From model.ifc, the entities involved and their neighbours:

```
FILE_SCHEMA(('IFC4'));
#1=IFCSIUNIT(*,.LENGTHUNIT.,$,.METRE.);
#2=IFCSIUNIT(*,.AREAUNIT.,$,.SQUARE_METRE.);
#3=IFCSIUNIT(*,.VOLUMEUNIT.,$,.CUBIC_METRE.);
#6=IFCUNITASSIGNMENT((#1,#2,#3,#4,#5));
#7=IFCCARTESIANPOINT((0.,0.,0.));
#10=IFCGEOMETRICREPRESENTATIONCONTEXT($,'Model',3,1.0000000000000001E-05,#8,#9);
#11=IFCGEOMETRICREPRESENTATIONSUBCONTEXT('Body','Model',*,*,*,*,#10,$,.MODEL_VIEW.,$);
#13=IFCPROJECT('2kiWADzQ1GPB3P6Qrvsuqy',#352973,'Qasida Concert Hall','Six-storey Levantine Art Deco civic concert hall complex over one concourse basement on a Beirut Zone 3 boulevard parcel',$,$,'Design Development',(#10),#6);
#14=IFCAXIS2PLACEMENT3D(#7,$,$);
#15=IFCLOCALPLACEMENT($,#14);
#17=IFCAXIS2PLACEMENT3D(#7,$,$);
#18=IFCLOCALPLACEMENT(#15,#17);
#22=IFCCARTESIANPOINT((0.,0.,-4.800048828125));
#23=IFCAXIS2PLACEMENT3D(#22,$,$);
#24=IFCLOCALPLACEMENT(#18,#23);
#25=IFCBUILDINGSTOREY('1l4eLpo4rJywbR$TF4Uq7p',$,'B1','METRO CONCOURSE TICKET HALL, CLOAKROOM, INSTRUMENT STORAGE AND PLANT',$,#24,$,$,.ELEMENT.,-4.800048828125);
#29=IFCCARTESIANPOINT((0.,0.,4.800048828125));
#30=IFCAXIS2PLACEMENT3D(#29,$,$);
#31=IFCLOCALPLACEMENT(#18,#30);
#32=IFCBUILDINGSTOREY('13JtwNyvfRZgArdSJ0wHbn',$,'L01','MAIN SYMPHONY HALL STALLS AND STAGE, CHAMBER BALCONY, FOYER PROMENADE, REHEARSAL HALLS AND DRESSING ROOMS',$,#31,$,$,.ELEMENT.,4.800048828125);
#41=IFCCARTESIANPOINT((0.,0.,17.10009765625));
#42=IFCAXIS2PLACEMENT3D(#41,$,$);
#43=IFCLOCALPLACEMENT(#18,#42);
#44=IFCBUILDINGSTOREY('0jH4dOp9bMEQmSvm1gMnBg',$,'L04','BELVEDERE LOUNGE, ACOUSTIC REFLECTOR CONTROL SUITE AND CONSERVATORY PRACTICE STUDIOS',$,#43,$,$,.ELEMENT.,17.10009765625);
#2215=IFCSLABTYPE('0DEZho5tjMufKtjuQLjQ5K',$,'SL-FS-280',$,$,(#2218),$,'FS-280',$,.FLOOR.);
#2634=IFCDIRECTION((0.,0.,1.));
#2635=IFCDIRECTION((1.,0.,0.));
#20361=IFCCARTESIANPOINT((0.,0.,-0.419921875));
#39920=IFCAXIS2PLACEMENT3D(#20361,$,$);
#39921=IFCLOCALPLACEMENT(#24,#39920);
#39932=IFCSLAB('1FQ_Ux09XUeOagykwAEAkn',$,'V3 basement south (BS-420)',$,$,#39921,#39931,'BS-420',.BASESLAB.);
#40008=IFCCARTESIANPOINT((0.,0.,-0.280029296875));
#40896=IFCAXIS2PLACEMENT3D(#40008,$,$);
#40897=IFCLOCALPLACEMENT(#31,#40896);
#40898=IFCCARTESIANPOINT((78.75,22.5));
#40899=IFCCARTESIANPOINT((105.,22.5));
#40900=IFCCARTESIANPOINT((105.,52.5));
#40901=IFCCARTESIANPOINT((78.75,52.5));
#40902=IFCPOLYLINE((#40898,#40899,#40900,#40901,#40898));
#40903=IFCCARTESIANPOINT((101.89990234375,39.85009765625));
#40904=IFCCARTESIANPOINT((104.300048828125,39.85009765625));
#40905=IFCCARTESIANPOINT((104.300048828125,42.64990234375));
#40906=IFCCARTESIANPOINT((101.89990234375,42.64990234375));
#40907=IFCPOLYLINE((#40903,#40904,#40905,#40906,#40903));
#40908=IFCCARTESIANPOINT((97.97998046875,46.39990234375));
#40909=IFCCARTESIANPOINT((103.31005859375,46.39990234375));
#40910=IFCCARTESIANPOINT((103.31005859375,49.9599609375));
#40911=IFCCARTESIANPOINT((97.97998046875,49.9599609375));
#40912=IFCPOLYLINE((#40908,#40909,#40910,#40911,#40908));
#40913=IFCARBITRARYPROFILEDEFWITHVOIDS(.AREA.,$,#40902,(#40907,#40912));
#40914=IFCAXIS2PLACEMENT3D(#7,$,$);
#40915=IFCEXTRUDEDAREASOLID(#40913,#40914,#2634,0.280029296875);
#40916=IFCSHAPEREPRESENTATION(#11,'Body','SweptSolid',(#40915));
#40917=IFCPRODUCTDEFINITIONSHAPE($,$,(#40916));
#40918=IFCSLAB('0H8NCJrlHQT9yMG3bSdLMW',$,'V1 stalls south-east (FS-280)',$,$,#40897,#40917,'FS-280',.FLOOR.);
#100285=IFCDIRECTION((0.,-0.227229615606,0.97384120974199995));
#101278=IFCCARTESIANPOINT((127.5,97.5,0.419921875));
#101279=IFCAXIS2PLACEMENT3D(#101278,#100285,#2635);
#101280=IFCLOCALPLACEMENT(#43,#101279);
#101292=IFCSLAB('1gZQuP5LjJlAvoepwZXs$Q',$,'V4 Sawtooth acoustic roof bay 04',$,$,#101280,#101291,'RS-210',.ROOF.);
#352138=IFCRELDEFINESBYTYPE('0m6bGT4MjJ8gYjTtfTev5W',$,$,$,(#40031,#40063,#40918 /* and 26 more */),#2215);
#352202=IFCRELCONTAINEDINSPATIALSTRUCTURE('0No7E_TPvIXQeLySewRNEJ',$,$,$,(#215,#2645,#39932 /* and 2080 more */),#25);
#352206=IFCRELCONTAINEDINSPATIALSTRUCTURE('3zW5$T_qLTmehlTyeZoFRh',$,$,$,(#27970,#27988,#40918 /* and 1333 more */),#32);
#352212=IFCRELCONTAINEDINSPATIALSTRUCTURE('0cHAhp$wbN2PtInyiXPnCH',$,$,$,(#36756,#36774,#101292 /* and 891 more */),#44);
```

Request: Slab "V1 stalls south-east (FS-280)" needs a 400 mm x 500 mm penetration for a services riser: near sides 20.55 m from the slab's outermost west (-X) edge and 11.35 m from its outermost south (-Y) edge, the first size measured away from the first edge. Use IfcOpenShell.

```python
import numpy as np
import ifcopenshell
import ifcopenshell.api.feature
import ifcopenshell.api.geometry
import ifcopenshell.api.root
import ifcopenshell.geom
import ifcopenshell.util.placement
import ifcopenshell.util.representation
import ifcopenshell.util.shape
import ifcopenshell.util.unit

model = ifcopenshell.open("model.ifc")
unit_scale = ifcopenshell.util.unit.calculate_unit_scale(model)
settings = ifcopenshell.geom.settings()


def volume(element):
    """Net volume in cubic metres, openings subtracted."""
    shape = ifcopenshell.geom.create_shape(settings, element)
    return ifcopenshell.util.shape.get_volume(shape.geometry)


slab = model.by_id(40918)
before = volume(slab)

# Extent in the slab's own axes, in metres. The edges named are its -X and -Y sides.
slab_shape = ifcopenshell.geom.create_shape(settings, slab)
vertices = ifcopenshell.util.shape.get_vertices(slab_shape.geometry)
x_min, y_min, bottom = vertices.min(axis=0)
top = vertices[:, 2].max()

opening = ifcopenshell.api.root.create_entity(model, ifc_class="IfcOpeningElement", name="Services riser opening", predefined_type="OPENING")
context = ifcopenshell.util.representation.get_context(model, "Model", "Body", "MODEL_VIEW")
width, depth = 0.4, 0.5
outline = [(0.0, 0.0), (width, 0.0), (width, depth), (0.0, depth), (0.0, 0.0)]
# Overshoot both faces by 50 mm so the cut is clean.
shape = ifcopenshell.api.geometry.add_slab_representation(
    model, context=context, depth=top - bottom + 0.1, polyline=outline
)
ifcopenshell.api.geometry.assign_representation(model, product=opening, representation=shape)

matrix = ifcopenshell.util.placement.get_local_placement(slab.ObjectPlacement)
matrix[:, 3] = matrix @ np.append(np.array([x_min + 20.55, y_min + 11.35, bottom - 0.05]) / unit_scale, 1.0)
ifcopenshell.api.geometry.edit_object_placement(model, product=opening, matrix=matrix, is_si=False)
ifcopenshell.api.feature.add_feature(model, feature=opening, element=slab)

after = volume(slab)

print(f"slab volume {before:.3f} -> {after:.3f} m3")

model.write("model_updated.ifc")
```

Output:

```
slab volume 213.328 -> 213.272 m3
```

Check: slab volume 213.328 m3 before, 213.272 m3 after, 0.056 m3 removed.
